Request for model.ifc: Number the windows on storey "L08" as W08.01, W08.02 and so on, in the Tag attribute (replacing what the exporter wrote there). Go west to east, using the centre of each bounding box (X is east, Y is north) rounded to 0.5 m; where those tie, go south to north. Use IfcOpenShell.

First a look at what the model holds.

```python
import ifcopenshell
import ifcopenshell.util.element
import ifcopenshell.util.placement

model = ifcopenshell.open("model.ifc")
print(model.schema)
storey = next(s for s in model.by_type("IfcBuildingStorey") if s.Name == "L08")
windows = [e for e in ifcopenshell.util.element.get_decomposition(storey) if e.is_a("IfcWindow")]
for e in sorted(windows, key=lambda e: e.id()):
    origin = ifcopenshell.util.placement.get_local_placement(e.ObjectPlacement)[:3, 3]
    print(e.id(), e.Tag, e.Name, origin.round(2) + 0.0, sep=" | ")
```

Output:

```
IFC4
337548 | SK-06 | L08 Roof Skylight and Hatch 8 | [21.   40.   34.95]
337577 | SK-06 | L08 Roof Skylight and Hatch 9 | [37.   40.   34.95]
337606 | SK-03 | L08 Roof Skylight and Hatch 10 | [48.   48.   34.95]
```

```python
import ifcopenshell
import ifcopenshell.geom
import ifcopenshell.util.element
import ifcopenshell.util.shape

model = ifcopenshell.open("model.ifc")
settings = ifcopenshell.geom.settings()
settings.set("use-world-coords", True)


def centre(element):
    shape = ifcopenshell.geom.create_shape(settings, element)
    return ifcopenshell.util.shape.get_bbox_centroid(shape.geometry)


storey = next(s for s in model.by_type("IfcBuildingStorey") if s.Name == "L08")
windows = [e for e in ifcopenshell.util.element.get_decomposition(storey) if e.is_a("IfcWindow")]

# Insertion points can sit at a corner or the storey origin, so sort by the geometry (in metres).
centres = {e: centre(e) for e in windows}
windows.sort(key=lambda e: (round(centres[e][0] / 0.5), centres[e][1]))

for i, e in enumerate(windows, start=1):
    number = f"W08.{i:02d}"
    e.Tag = number
    print(e.id(), number)

model.write("model_edited.ifc")
```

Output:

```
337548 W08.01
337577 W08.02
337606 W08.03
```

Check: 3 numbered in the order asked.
